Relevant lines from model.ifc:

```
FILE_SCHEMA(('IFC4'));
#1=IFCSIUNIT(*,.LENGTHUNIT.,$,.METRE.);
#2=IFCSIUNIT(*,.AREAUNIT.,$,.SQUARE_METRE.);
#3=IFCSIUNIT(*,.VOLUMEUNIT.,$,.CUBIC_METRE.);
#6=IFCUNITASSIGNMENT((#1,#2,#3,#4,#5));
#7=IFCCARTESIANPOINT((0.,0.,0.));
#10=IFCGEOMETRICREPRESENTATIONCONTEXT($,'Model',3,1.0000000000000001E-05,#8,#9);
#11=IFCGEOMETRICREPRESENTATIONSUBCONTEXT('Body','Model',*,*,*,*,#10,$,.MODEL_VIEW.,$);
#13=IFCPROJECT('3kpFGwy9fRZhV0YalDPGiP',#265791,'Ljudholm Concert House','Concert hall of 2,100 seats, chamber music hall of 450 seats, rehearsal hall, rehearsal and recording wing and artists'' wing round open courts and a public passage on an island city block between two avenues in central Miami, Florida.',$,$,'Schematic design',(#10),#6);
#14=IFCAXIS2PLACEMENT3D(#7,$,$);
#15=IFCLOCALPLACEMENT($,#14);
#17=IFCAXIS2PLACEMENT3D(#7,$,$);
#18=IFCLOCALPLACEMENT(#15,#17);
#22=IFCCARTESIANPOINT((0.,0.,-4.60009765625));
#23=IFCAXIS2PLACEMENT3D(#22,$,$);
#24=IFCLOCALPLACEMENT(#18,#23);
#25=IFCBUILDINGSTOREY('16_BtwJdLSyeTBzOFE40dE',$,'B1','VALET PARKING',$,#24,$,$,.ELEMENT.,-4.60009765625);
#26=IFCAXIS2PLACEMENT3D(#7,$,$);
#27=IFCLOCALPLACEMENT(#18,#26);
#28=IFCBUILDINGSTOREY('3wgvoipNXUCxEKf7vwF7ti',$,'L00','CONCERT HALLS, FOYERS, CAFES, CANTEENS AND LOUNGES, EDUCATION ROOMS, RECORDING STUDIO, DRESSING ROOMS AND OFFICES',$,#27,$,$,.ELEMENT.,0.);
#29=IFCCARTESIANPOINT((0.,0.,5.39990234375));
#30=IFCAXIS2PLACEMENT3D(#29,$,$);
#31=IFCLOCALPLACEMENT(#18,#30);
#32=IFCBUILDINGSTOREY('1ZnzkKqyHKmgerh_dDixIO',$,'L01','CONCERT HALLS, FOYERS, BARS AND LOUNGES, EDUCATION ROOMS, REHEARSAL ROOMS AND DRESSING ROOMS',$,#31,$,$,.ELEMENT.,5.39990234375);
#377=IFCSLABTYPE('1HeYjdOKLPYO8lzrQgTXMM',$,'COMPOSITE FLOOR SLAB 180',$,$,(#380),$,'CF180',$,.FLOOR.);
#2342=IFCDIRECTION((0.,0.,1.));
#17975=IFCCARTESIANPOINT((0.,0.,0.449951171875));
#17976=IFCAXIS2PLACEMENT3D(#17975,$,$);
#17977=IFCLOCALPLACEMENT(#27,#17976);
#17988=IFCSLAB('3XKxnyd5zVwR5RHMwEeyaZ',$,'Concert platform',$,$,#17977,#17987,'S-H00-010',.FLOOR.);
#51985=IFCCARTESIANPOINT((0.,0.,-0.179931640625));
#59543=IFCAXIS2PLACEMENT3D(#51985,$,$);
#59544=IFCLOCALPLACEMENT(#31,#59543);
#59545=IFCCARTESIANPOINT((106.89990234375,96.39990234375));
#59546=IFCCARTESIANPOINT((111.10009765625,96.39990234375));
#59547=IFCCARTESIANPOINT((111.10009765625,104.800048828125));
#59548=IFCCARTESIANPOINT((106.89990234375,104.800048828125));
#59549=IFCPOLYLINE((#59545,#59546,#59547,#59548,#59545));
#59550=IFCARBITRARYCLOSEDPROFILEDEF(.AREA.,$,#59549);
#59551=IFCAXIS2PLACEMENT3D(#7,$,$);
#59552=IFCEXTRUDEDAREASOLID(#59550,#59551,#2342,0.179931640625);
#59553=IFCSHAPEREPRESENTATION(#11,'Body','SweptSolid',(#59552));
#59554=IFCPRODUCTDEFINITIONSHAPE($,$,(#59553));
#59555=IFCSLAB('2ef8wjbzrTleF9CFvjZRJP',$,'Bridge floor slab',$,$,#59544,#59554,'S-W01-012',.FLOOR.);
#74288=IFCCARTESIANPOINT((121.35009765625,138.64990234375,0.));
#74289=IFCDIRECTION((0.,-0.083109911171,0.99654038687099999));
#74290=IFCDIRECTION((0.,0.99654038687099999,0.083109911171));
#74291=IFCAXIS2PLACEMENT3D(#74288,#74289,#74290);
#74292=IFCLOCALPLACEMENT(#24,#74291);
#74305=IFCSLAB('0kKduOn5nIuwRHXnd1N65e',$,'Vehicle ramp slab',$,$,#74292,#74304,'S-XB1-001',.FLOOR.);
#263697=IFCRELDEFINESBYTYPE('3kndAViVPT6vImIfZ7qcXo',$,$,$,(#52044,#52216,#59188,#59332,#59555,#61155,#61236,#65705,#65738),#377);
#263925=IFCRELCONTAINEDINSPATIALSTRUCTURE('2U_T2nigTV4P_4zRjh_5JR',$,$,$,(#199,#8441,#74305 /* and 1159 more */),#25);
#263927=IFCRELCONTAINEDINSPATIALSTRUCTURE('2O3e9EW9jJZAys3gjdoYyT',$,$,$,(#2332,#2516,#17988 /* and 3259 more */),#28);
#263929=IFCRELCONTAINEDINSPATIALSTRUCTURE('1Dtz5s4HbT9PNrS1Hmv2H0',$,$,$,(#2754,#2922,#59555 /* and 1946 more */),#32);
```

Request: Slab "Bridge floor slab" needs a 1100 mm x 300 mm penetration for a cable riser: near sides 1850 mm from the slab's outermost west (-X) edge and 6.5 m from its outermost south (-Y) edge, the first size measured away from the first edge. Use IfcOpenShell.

```python
import numpy as np
import ifcopenshell
import ifcopenshell.api.feature
import ifcopenshell.api.geometry
import ifcopenshell.api.root
import ifcopenshell.geom
import ifcopenshell.util.placement
import ifcopenshell.util.representation
import ifcopenshell.util.shape
import ifcopenshell.util.unit

model = ifcopenshell.open("model.ifc")
unit_scale = ifcopenshell.util.unit.calculate_unit_scale(model)
settings = ifcopenshell.geom.settings()


def volume(element):
    """Net volume in cubic metres, openings subtracted."""
    shape = ifcopenshell.geom.create_shape(settings, element)
    return ifcopenshell.util.shape.get_volume(shape.geometry)


slab = model.by_guid("2ef8wjbzrTleF9CFvjZRJP")
before = volume(slab)

# Extent in the slab's own axes, in metres. The edges named are its -X and -Y sides.
slab_shape = ifcopenshell.geom.create_shape(settings, slab)
vertices = ifcopenshell.util.shape.get_vertices(slab_shape.geometry)
x_min, y_min, bottom = vertices.min(axis=0)
top = vertices[:, 2].max()

opening = ifcopenshell.api.root.create_entity(model, ifc_class="IfcOpeningElement", name="Cable riser opening", predefined_type="OPENING")
context = ifcopenshell.util.representation.get_context(model, "Model", "Body", "MODEL_VIEW")
width, depth = 1.1, 0.3
outline = [(0.0, 0.0), (width, 0.0), (width, depth), (0.0, depth), (0.0, 0.0)]
# Overshoot both faces by 50 mm so the cut is clean.
shape = ifcopenshell.api.geometry.add_slab_representation(
    model, context=context, depth=top - bottom + 0.1, polyline=outline
)
ifcopenshell.api.geometry.assign_representation(model, product=opening, representation=shape)

matrix = ifcopenshell.util.placement.get_local_placement(slab.ObjectPlacement)
matrix[:, 3] = matrix @ np.append(np.array([x_min + 1.85, y_min + 6.5, bottom - 0.05]) / unit_scale, 1.0)
ifcopenshell.api.geometry.edit_object_placement(model, product=opening, matrix=matrix, is_si=False)
ifcopenshell.api.feature.add_feature(model, feature=opening, element=slab)

after = volume(slab)

print(f"slab volume {before:.3f} -> {after:.3f} m3")

model.write("model_v2.ifc")
```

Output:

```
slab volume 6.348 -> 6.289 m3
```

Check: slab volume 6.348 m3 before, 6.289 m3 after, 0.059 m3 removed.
